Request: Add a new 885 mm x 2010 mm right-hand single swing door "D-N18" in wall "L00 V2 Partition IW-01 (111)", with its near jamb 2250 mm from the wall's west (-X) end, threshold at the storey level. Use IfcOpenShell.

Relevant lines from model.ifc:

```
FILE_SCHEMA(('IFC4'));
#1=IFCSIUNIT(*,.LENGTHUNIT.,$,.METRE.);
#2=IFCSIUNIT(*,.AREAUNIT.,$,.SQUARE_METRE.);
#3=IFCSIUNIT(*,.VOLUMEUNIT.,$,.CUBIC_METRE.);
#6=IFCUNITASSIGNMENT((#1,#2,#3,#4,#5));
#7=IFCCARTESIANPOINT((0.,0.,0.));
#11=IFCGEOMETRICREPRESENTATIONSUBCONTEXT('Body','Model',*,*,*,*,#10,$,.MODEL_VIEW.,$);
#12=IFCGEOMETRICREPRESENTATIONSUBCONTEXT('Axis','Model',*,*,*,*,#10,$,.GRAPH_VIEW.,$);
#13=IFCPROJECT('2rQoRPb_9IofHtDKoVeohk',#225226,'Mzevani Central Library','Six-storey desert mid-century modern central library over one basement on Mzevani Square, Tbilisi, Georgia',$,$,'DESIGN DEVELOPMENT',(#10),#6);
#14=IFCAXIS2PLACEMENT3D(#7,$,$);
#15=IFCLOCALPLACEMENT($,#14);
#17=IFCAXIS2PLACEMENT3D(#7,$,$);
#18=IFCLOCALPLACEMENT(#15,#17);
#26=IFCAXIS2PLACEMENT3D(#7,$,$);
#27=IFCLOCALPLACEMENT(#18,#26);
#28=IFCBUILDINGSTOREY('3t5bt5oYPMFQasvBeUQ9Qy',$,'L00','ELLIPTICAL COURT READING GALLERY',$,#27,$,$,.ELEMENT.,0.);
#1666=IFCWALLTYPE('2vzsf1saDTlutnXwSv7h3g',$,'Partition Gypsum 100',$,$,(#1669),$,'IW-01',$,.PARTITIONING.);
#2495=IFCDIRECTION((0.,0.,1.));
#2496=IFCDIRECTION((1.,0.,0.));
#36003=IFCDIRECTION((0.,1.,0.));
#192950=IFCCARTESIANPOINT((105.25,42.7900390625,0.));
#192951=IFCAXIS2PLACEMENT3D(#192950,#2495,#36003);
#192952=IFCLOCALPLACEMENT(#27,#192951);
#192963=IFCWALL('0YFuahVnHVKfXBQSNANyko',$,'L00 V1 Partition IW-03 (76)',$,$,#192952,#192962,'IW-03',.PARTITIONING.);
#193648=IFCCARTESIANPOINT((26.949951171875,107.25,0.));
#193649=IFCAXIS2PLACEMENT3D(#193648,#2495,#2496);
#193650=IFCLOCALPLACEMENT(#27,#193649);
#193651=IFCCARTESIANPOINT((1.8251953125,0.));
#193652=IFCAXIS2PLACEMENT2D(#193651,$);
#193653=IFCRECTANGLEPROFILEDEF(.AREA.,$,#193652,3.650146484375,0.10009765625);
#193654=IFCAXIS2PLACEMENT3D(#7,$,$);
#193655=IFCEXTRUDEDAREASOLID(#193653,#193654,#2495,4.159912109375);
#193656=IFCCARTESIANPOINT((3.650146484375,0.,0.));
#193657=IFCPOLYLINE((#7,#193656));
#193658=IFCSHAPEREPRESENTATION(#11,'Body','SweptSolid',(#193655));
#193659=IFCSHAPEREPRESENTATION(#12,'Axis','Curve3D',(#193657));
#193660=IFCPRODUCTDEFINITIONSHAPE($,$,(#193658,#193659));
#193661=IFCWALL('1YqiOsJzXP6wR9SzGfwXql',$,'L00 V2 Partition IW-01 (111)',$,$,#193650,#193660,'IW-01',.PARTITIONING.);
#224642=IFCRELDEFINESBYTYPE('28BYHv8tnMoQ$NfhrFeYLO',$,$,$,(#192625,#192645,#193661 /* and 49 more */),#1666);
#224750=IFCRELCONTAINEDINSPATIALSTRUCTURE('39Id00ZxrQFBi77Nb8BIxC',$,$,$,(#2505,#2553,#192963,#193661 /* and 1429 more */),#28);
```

```python
import numpy as np
import ifcopenshell
import ifcopenshell.api.feature
import ifcopenshell.api.geometry
import ifcopenshell.api.root
import ifcopenshell.api.spatial
import ifcopenshell.geom
import ifcopenshell.util.element
import ifcopenshell.util.placement
import ifcopenshell.util.representation
import ifcopenshell.util.shape
import ifcopenshell.util.unit

model = ifcopenshell.open("model.ifc")
unit_scale = ifcopenshell.util.unit.calculate_unit_scale(model)
settings = ifcopenshell.geom.settings()


def volume(element):
    """Net volume in cubic metres, openings subtracted."""
    shape = ifcopenshell.geom.create_shape(settings, element)
    return ifcopenshell.util.shape.get_volume(shape.geometry)


wall = model.by_guid("1YqiOsJzXP6wR9SzGfwXql")
storey = ifcopenshell.util.element.get_container(wall, ifc_class="IfcBuildingStorey")
context = ifcopenshell.util.representation.get_context(model, "Model", "Body", "MODEL_VIEW")
before = volume(wall)

width, height, from_end, sill = 0.885, 2.01, 2.25, 0.0  # metres

# The wall runs along its own X axis, and the end named is its -X end.
wall_shape = ifcopenshell.geom.create_shape(settings, wall)
x, y, z = ifcopenshell.util.shape.get_vertices(wall_shape.geometry).T
start = x.min() + from_end
face, thickness = float(y.min()), float(y.max() - y.min())
wall_matrix = ifcopenshell.util.placement.get_local_placement(wall.ObjectPlacement)
level = ifcopenshell.util.placement.get_local_placement(storey.ObjectPlacement)[2, 3]


def in_wall(x, y):
    """Placement at x, y metres in the wall's axes, at sill height."""
    matrix = wall_matrix.copy()
    matrix[:, 3] = wall_matrix @ np.array([x / unit_scale, y / unit_scale, 0.0, 1.0])
    matrix[2, 3] = level + sill / unit_scale
    return matrix


# Opening: a box that overshoots both wall faces by 50 mm.
opening = ifcopenshell.api.root.create_entity(model, ifc_class="IfcOpeningElement", predefined_type="OPENING")
box = ifcopenshell.api.geometry.add_wall_representation(
    model, context=context, length=width, height=height, thickness=thickness + 0.1
)
ifcopenshell.api.geometry.assign_representation(model, product=opening, representation=box)
ifcopenshell.api.geometry.edit_object_placement(model, product=opening, matrix=in_wall(start, face - 0.05), is_si=False)
ifcopenshell.api.feature.add_feature(model, feature=opening, element=wall)

door = ifcopenshell.api.root.create_entity(model, ifc_class="IfcDoor", name="D-N18", predefined_type="DOOR")
door.OverallWidth, door.OverallHeight = width / unit_scale, height / unit_scale
door.OperationType = "SINGLE_SWING_RIGHT"
body = ifcopenshell.api.geometry.add_door_representation(
    model,
    context=context,
    overall_width=door.OverallWidth,
    overall_height=door.OverallHeight,
    operation_type="SINGLE_SWING_RIGHT",
    lining_properties={"LiningDepth": thickness / unit_scale, "ThresholdDepth": thickness / unit_scale},
)
ifcopenshell.api.geometry.assign_representation(model, product=door, representation=body)
ifcopenshell.api.spatial.assign_container(model, products=[door], relating_structure=storey)
ifcopenshell.api.feature.add_filling(model, opening=opening, element=door)

# The lining spans the wall, so the door starts at the wall face.
ifcopenshell.api.geometry.edit_object_placement(model, product=door, matrix=in_wall(start, face), is_si=False)

after = volume(wall)

print(f"wall volume {before:.3f} -> {after:.3f} m3")

model.write("model_rev.ifc")
```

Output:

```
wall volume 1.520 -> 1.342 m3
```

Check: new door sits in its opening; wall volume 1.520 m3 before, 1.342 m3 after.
